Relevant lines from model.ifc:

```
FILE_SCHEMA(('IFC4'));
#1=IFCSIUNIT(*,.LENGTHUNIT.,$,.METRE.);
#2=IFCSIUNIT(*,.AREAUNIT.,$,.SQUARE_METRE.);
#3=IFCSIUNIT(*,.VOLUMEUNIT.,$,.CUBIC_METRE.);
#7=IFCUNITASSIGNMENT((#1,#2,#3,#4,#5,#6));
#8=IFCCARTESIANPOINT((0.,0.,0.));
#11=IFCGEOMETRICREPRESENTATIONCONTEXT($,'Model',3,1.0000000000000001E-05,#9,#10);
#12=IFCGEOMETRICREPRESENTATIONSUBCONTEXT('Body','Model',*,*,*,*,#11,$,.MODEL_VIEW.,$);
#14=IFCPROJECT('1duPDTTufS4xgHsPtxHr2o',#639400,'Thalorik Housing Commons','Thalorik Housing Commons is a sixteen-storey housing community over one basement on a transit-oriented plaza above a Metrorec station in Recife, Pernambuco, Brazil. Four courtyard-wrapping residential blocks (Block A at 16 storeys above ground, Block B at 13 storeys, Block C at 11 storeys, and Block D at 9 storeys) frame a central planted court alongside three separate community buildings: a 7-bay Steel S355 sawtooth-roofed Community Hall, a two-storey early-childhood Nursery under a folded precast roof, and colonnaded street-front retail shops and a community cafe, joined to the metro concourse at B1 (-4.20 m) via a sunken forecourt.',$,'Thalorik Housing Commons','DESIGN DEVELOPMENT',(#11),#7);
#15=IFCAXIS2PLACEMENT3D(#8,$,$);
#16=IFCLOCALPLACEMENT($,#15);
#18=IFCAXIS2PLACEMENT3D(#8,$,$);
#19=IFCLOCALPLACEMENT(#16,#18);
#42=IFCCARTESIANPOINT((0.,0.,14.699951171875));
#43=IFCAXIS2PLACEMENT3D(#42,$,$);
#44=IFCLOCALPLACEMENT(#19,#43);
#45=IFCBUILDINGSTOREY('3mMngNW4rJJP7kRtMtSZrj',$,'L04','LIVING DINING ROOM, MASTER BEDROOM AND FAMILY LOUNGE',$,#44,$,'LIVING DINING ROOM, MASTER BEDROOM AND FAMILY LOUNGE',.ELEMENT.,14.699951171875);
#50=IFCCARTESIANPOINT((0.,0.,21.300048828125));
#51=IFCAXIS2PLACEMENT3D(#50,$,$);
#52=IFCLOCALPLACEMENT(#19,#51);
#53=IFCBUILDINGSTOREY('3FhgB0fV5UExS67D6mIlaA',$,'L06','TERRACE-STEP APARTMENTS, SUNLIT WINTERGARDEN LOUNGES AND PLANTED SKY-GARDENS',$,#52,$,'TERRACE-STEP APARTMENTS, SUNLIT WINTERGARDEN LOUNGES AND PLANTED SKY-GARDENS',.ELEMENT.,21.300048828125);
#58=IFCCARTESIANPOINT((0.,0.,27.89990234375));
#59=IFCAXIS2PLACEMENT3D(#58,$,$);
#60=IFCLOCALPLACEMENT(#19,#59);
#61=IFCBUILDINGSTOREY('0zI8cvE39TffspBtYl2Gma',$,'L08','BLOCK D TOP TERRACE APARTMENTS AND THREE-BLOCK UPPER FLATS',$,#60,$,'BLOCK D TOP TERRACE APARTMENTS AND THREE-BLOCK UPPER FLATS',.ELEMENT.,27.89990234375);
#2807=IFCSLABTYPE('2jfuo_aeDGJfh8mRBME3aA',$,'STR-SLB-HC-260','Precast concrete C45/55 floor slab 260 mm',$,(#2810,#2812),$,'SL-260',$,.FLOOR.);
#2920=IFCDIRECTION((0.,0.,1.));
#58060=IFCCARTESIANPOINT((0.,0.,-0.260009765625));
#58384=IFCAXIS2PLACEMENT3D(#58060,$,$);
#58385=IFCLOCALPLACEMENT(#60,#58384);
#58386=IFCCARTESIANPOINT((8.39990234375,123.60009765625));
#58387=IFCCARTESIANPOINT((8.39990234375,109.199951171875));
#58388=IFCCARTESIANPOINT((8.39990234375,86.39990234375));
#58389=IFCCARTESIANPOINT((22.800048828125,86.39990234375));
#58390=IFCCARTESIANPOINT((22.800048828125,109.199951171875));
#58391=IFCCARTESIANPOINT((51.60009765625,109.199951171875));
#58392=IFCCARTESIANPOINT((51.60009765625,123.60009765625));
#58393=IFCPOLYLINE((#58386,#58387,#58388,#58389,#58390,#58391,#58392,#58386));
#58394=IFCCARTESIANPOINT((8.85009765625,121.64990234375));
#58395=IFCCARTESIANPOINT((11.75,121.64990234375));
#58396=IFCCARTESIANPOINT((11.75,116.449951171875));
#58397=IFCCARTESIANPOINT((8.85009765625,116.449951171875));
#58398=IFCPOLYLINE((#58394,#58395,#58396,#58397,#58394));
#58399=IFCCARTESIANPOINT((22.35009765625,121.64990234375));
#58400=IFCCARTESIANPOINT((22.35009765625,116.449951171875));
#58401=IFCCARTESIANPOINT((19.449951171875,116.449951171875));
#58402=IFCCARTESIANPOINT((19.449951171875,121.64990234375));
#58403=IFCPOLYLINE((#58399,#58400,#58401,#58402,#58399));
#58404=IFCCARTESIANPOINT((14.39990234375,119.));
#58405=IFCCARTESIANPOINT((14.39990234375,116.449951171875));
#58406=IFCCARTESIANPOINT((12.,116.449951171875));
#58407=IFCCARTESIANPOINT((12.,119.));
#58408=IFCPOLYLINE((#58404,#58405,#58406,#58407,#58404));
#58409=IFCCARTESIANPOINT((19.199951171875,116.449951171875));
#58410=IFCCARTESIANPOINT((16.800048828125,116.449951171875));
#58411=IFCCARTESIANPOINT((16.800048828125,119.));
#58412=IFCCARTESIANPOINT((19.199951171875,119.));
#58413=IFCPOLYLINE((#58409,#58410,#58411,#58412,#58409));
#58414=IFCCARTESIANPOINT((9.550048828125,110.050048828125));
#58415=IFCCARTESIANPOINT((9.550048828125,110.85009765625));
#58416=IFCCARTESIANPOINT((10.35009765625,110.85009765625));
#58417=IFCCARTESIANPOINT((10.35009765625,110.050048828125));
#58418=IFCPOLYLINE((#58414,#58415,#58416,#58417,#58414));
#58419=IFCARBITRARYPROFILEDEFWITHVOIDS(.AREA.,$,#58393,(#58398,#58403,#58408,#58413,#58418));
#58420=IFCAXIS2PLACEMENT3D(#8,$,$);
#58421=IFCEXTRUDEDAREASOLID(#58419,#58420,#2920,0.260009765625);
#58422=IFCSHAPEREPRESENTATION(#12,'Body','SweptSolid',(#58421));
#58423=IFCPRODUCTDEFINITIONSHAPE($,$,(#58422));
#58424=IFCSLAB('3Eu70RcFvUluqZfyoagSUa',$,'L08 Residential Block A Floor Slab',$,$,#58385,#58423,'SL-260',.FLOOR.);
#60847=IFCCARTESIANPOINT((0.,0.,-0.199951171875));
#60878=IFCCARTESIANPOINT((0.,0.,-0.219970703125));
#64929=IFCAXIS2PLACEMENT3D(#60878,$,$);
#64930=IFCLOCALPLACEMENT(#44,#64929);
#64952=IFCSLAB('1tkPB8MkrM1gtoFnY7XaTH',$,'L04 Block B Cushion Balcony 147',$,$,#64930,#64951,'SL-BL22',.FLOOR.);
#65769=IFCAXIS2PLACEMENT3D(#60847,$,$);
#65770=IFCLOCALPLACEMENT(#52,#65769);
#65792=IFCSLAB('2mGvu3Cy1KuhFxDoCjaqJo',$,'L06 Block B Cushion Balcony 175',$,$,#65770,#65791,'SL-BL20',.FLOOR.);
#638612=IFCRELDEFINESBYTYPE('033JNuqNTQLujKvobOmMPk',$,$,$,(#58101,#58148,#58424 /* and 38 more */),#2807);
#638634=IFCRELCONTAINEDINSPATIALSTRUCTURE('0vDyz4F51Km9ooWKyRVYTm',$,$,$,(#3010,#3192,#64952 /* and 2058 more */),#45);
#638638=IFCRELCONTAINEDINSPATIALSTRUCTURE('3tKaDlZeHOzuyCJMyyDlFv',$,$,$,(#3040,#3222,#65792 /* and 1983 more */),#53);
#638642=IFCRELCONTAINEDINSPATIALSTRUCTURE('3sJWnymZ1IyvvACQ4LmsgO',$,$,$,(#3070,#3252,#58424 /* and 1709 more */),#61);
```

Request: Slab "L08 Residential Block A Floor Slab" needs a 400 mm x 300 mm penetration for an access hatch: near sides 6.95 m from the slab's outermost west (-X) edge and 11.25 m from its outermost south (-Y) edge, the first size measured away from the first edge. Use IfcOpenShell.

```python
import numpy as np
import ifcopenshell
import ifcopenshell.api.feature
import ifcopenshell.api.geometry
import ifcopenshell.api.root
import ifcopenshell.geom
import ifcopenshell.util.placement
import ifcopenshell.util.representation
import ifcopenshell.util.shape
import ifcopenshell.util.unit

model = ifcopenshell.open("model.ifc")
unit_scale = ifcopenshell.util.unit.calculate_unit_scale(model)
settings = ifcopenshell.geom.settings()


def volume(element):
    """Net volume in cubic metres, openings subtracted."""
    shape = ifcopenshell.geom.create_shape(settings, element)
    return ifcopenshell.util.shape.get_volume(shape.geometry)


slab = model.by_guid("3Eu70RcFvUluqZfyoagSUa")
before = volume(slab)

# Extent in the slab's own axes, in metres. The edges named are its -X and -Y sides.
slab_shape = ifcopenshell.geom.create_shape(settings, slab)
vertices = ifcopenshell.util.shape.get_vertices(slab_shape.geometry)
x_min, y_min, bottom = vertices.min(axis=0)
top = vertices[:, 2].max()

opening = ifcopenshell.api.root.create_entity(model, ifc_class="IfcOpeningElement", name="Access hatch opening", predefined_type="OPENING")
context = ifcopenshell.util.representation.get_context(model, "Model", "Body", "MODEL_VIEW")
width, depth = 0.4, 0.3
outline = [(0.0, 0.0), (width, 0.0), (width, depth), (0.0, depth), (0.0, 0.0)]
# Overshoot both faces by 50 mm so the cut is clean.
shape = ifcopenshell.api.geometry.add_slab_representation(
    model, context=context, depth=top - bottom + 0.1, polyline=outline
)
ifcopenshell.api.geometry.assign_representation(model, product=opening, representation=shape)

matrix = ifcopenshell.util.placement.get_local_placement(slab.ObjectPlacement)
matrix[:, 3] = matrix @ np.append(np.array([x_min + 6.95, y_min + 11.25, bottom - 0.05]) / unit_scale, 1.0)
ifcopenshell.api.geometry.edit_object_placement(model, product=opening, matrix=matrix, is_si=False)
ifcopenshell.api.feature.add_feature(model, feature=opening, element=slab)

after = volume(slab)

print(f"slab volume {before:.3f} -> {after:.3f} m3")

model.write("model_v2.ifc")
```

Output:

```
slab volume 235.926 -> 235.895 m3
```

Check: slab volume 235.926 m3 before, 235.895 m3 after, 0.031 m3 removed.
